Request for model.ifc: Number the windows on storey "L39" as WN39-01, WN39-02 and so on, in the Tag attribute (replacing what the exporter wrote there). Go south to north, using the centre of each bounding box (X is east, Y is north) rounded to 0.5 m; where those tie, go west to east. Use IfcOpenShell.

First a look at what the model holds.

```python
import ifcopenshell
import ifcopenshell.util.element
import ifcopenshell.util.placement

model = ifcopenshell.open("model.ifc")
print(model.schema)
storey = next(s for s in model.by_type("IfcBuildingStorey") if s.Name == "L39")
windows = [e for e in ifcopenshell.util.element.get_decomposition(storey) if e.is_a("IfcWindow")]
for e in sorted(windows, key=lambda e: e.id()):
    origin = ifcopenshell.util.placement.get_local_placement(e.ObjectPlacement)[:3, 3]
    print(e.id(), e.Tag, e.Name, origin.round(2) + 0.0, sep=" | ")
```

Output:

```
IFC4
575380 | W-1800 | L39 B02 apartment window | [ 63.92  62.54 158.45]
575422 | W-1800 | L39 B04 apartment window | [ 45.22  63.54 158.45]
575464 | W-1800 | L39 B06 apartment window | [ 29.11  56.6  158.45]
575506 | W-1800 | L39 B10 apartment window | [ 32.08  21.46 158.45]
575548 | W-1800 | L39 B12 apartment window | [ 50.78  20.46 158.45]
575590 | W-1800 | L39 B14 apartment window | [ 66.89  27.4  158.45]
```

```python
import ifcopenshell
import ifcopenshell.geom
import ifcopenshell.util.element
import ifcopenshell.util.shape

model = ifcopenshell.open("model.ifc")
settings = ifcopenshell.geom.settings()
settings.set("use-world-coords", True)


def centre(element):
    shape = ifcopenshell.geom.create_shape(settings, element)
    return ifcopenshell.util.shape.get_bbox_centroid(shape.geometry)


storey = next(s for s in model.by_type("IfcBuildingStorey") if s.Name == "L39")
windows = [e for e in ifcopenshell.util.element.get_decomposition(storey) if e.is_a("IfcWindow")]

# Insertion points can sit at a corner or the storey origin, so sort by the geometry (in metres).
centres = {e: centre(e) for e in windows}
windows.sort(key=lambda e: (round(centres[e][1] / 0.5), centres[e][0]))

for i, e in enumerate(windows, start=1):
    number = f"WN39-{i:02d}"
    e.Tag = number
    print(e.id(), number)

model.write("model_v2.ifc")
```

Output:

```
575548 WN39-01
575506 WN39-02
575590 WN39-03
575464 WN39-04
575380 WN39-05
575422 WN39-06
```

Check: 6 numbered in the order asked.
